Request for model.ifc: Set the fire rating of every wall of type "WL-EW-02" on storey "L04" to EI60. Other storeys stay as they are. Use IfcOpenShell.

First a look at what the model holds.

```python
import ifcopenshell
import ifcopenshell.util.element

model = ifcopenshell.open("model.ifc")
print(model.schema)
storey = next(s for s in model.by_type("IfcBuildingStorey") if s.Name == "L04")
walls = [e for e in ifcopenshell.util.element.get_decomposition(storey) if e.is_a("IfcWall")]
seen = {}
for e in walls:
    element_type = ifcopenshell.util.element.get_type(e)
    key = (element_type.Name if element_type != e and element_type else None, ifcopenshell.util.element.get_pset(e, "Pset_WallCommon", "FireRating"))
    seen[key] = seen.get(key, 0) + 1
for (name, value), count in sorted(seen.items(), key=str):
    print(count, "x", name, "|", value)
```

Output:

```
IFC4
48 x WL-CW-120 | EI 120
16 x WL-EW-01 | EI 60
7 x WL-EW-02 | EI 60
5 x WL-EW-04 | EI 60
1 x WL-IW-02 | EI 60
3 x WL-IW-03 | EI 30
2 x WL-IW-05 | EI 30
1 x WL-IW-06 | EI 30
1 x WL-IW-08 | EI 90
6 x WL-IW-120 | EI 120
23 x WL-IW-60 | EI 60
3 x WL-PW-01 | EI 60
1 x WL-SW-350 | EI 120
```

```python
import ifcopenshell
import ifcopenshell.api.pset
import ifcopenshell.util.element

model = ifcopenshell.open("model.ifc")

storey = next(s for s in model.by_type("IfcBuildingStorey") if s.Name == "L04")
walls = [e for e in ifcopenshell.util.element.get_decomposition(storey) if e.is_a("IfcWall")]

count = 0
for e in walls:
    element_type = ifcopenshell.util.element.get_type(e)
    if element_type in (None, e) or element_type.Name != "WL-EW-02":
        continue
    # add_pset returns the element's existing set when there is one.
    pset = ifcopenshell.api.pset.add_pset(model, product=e, name="Pset_WallCommon")
    ifcopenshell.api.pset.edit_pset(model, pset=pset, properties={"FireRating": "EI60"})
    count += 1

print(count, "walls updated")

model.write("model_rev.ifc")
```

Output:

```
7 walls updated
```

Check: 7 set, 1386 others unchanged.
